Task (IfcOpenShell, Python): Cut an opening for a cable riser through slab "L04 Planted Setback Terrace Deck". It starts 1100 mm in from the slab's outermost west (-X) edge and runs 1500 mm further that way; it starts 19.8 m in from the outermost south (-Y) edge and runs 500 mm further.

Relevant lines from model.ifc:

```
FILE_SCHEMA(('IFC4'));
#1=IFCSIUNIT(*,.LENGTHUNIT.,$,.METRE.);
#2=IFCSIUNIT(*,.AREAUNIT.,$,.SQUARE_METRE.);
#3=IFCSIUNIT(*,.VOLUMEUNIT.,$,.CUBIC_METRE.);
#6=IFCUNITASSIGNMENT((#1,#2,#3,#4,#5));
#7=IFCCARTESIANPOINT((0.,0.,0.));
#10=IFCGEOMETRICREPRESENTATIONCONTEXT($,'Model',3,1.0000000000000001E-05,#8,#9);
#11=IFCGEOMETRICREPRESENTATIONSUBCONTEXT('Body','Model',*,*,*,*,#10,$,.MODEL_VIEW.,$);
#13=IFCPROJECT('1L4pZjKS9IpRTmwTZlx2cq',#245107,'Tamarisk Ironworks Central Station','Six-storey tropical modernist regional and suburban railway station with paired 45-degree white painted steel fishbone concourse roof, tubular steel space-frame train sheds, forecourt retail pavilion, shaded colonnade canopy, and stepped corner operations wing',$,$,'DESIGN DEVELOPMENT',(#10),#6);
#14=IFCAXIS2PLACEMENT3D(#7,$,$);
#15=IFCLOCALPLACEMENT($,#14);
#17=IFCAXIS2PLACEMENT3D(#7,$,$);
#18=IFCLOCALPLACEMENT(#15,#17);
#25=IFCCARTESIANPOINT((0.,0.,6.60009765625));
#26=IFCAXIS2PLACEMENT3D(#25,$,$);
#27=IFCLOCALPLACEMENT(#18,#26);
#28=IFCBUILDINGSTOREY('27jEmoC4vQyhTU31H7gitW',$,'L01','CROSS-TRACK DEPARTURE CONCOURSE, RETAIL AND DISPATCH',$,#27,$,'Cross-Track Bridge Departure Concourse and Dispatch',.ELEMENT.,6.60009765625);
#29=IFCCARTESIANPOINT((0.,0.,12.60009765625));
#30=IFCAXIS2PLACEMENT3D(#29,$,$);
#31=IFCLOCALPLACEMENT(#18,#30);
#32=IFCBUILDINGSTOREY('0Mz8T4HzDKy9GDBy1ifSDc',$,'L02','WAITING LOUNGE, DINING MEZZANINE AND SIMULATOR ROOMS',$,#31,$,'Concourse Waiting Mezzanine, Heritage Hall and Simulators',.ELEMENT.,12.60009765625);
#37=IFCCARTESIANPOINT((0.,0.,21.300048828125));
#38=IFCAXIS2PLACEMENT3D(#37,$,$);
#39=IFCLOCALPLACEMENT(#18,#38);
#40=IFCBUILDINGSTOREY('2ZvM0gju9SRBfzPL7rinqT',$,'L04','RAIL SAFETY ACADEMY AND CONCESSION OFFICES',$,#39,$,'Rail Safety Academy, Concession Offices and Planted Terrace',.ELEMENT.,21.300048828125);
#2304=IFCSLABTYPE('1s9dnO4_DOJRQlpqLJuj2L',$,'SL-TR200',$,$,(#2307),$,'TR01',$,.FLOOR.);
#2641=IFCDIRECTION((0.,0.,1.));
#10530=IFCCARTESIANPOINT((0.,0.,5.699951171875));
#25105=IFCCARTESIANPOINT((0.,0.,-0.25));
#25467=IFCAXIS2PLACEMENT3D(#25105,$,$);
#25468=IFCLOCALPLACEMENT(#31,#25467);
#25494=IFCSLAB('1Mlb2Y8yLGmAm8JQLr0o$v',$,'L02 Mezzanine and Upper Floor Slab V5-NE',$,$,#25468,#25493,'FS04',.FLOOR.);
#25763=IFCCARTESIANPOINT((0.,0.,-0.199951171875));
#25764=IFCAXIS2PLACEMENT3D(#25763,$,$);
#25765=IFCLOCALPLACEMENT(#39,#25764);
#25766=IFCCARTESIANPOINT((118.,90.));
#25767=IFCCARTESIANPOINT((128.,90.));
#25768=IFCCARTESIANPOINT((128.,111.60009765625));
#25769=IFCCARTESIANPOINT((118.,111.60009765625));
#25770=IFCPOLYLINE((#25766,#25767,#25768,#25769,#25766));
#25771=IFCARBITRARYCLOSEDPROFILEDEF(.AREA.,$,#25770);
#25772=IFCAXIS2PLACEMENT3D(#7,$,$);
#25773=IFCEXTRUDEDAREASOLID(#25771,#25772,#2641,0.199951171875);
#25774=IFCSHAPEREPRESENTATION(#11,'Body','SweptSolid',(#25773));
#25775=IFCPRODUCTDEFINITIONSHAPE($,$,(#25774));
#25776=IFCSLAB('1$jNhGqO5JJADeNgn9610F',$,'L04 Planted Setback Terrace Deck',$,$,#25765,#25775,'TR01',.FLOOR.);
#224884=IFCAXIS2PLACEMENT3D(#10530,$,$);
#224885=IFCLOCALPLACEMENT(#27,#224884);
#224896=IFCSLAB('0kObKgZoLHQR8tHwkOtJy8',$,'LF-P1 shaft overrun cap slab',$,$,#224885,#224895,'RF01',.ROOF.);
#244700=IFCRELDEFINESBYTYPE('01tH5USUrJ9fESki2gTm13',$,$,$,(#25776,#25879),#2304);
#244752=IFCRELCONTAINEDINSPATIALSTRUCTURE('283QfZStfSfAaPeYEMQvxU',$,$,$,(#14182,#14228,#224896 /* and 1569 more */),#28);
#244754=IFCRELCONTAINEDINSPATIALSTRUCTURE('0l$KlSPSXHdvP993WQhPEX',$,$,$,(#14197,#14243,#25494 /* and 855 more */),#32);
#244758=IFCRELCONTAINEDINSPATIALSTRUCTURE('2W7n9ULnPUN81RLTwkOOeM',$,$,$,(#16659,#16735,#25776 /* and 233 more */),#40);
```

```python
import numpy as np
import ifcopenshell
import ifcopenshell.api.feature
import ifcopenshell.api.geometry
import ifcopenshell.api.root
import ifcopenshell.geom
import ifcopenshell.util.placement
import ifcopenshell.util.representation
import ifcopenshell.util.shape
import ifcopenshell.util.unit

model = ifcopenshell.open("model.ifc")
unit_scale = ifcopenshell.util.unit.calculate_unit_scale(model)
settings = ifcopenshell.geom.settings()


def volume(element):
    """Net volume in cubic metres, openings subtracted."""
    shape = ifcopenshell.geom.create_shape(settings, element)
    return ifcopenshell.util.shape.get_volume(shape.geometry)


slab = model.by_guid("1$jNhGqO5JJADeNgn9610F")
before = volume(slab)

# Extent in the slab's own axes, in metres. The edges named are its -X and -Y sides.
slab_shape = ifcopenshell.geom.create_shape(settings, slab)
vertices = ifcopenshell.util.shape.get_vertices(slab_shape.geometry)
x_min, y_min, bottom = vertices.min(axis=0)
top = vertices[:, 2].max()

opening = ifcopenshell.api.root.create_entity(model, ifc_class="IfcOpeningElement", name="Cable riser opening", predefined_type="OPENING")
context = ifcopenshell.util.representation.get_context(model, "Model", "Body", "MODEL_VIEW")
width, depth = 1.5, 0.5
outline = [(0.0, 0.0), (width, 0.0), (width, depth), (0.0, depth), (0.0, 0.0)]
# Overshoot both faces by 50 mm so the cut is clean.
shape = ifcopenshell.api.geometry.add_slab_representation(
    model, context=context, depth=top - bottom + 0.1, polyline=outline
)
ifcopenshell.api.geometry.assign_representation(model, product=opening, representation=shape)

matrix = ifcopenshell.util.placement.get_local_placement(slab.ObjectPlacement)
matrix[:, 3] = matrix @ np.append(np.array([x_min + 1.1, y_min + 19.8, bottom - 0.05]) / unit_scale, 1.0)
ifcopenshell.api.geometry.edit_object_placement(model, product=opening, matrix=matrix, is_si=False)
ifcopenshell.api.feature.add_feature(model, feature=opening, element=slab)

after = volume(slab)

print(f"slab volume {before:.3f} -> {after:.3f} m3")

model.write("model_rev.ifc")
```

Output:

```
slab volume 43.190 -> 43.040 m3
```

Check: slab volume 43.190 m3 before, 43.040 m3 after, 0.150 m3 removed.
